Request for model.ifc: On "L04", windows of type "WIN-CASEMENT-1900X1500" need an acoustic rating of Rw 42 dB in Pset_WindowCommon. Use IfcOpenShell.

First a look at what the model holds.

```python
import ifcopenshell
import ifcopenshell.util.element

model = ifcopenshell.open("model.ifc")
print(model.schema)
storey = next(s for s in model.by_type("IfcBuildingStorey") if s.Name == "L04")
windows = [e for e in ifcopenshell.util.element.get_decomposition(storey) if e.is_a("IfcWindow")]
seen = {}
for e in windows:
    element_type = ifcopenshell.util.element.get_type(e)
    key = (element_type.Name if element_type != e and element_type else None, ifcopenshell.util.element.get_pset(e, "Pset_WindowCommon", "AcousticRating"))
    seen[key] = seen.get(key, 0) + 1
for (name, value), count in sorted(seen.items(), key=str):
    print(count, "x", name, "|", value)
```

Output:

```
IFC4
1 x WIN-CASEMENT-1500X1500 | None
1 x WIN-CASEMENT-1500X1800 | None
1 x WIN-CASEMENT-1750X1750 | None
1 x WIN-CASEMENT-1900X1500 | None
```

```python
import ifcopenshell
import ifcopenshell.api.pset
import ifcopenshell.util.element

model = ifcopenshell.open("model.ifc")

storey = next(s for s in model.by_type("IfcBuildingStorey") if s.Name == "L04")
windows = [e for e in ifcopenshell.util.element.get_decomposition(storey) if e.is_a("IfcWindow")]

count = 0
for e in windows:
    element_type = ifcopenshell.util.element.get_type(e)
    if element_type in (None, e) or element_type.Name != "WIN-CASEMENT-1900X1500":
        continue
    # add_pset returns the element's existing set when there is one.
    pset = ifcopenshell.api.pset.add_pset(model, product=e, name="Pset_WindowCommon")
    ifcopenshell.api.pset.edit_pset(model, pset=pset, properties={"AcousticRating": "Rw 42 dB"})
    count += 1

print(count, "windows updated")

model.write("model_v2.ifc")
```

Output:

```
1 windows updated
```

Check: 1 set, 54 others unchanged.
